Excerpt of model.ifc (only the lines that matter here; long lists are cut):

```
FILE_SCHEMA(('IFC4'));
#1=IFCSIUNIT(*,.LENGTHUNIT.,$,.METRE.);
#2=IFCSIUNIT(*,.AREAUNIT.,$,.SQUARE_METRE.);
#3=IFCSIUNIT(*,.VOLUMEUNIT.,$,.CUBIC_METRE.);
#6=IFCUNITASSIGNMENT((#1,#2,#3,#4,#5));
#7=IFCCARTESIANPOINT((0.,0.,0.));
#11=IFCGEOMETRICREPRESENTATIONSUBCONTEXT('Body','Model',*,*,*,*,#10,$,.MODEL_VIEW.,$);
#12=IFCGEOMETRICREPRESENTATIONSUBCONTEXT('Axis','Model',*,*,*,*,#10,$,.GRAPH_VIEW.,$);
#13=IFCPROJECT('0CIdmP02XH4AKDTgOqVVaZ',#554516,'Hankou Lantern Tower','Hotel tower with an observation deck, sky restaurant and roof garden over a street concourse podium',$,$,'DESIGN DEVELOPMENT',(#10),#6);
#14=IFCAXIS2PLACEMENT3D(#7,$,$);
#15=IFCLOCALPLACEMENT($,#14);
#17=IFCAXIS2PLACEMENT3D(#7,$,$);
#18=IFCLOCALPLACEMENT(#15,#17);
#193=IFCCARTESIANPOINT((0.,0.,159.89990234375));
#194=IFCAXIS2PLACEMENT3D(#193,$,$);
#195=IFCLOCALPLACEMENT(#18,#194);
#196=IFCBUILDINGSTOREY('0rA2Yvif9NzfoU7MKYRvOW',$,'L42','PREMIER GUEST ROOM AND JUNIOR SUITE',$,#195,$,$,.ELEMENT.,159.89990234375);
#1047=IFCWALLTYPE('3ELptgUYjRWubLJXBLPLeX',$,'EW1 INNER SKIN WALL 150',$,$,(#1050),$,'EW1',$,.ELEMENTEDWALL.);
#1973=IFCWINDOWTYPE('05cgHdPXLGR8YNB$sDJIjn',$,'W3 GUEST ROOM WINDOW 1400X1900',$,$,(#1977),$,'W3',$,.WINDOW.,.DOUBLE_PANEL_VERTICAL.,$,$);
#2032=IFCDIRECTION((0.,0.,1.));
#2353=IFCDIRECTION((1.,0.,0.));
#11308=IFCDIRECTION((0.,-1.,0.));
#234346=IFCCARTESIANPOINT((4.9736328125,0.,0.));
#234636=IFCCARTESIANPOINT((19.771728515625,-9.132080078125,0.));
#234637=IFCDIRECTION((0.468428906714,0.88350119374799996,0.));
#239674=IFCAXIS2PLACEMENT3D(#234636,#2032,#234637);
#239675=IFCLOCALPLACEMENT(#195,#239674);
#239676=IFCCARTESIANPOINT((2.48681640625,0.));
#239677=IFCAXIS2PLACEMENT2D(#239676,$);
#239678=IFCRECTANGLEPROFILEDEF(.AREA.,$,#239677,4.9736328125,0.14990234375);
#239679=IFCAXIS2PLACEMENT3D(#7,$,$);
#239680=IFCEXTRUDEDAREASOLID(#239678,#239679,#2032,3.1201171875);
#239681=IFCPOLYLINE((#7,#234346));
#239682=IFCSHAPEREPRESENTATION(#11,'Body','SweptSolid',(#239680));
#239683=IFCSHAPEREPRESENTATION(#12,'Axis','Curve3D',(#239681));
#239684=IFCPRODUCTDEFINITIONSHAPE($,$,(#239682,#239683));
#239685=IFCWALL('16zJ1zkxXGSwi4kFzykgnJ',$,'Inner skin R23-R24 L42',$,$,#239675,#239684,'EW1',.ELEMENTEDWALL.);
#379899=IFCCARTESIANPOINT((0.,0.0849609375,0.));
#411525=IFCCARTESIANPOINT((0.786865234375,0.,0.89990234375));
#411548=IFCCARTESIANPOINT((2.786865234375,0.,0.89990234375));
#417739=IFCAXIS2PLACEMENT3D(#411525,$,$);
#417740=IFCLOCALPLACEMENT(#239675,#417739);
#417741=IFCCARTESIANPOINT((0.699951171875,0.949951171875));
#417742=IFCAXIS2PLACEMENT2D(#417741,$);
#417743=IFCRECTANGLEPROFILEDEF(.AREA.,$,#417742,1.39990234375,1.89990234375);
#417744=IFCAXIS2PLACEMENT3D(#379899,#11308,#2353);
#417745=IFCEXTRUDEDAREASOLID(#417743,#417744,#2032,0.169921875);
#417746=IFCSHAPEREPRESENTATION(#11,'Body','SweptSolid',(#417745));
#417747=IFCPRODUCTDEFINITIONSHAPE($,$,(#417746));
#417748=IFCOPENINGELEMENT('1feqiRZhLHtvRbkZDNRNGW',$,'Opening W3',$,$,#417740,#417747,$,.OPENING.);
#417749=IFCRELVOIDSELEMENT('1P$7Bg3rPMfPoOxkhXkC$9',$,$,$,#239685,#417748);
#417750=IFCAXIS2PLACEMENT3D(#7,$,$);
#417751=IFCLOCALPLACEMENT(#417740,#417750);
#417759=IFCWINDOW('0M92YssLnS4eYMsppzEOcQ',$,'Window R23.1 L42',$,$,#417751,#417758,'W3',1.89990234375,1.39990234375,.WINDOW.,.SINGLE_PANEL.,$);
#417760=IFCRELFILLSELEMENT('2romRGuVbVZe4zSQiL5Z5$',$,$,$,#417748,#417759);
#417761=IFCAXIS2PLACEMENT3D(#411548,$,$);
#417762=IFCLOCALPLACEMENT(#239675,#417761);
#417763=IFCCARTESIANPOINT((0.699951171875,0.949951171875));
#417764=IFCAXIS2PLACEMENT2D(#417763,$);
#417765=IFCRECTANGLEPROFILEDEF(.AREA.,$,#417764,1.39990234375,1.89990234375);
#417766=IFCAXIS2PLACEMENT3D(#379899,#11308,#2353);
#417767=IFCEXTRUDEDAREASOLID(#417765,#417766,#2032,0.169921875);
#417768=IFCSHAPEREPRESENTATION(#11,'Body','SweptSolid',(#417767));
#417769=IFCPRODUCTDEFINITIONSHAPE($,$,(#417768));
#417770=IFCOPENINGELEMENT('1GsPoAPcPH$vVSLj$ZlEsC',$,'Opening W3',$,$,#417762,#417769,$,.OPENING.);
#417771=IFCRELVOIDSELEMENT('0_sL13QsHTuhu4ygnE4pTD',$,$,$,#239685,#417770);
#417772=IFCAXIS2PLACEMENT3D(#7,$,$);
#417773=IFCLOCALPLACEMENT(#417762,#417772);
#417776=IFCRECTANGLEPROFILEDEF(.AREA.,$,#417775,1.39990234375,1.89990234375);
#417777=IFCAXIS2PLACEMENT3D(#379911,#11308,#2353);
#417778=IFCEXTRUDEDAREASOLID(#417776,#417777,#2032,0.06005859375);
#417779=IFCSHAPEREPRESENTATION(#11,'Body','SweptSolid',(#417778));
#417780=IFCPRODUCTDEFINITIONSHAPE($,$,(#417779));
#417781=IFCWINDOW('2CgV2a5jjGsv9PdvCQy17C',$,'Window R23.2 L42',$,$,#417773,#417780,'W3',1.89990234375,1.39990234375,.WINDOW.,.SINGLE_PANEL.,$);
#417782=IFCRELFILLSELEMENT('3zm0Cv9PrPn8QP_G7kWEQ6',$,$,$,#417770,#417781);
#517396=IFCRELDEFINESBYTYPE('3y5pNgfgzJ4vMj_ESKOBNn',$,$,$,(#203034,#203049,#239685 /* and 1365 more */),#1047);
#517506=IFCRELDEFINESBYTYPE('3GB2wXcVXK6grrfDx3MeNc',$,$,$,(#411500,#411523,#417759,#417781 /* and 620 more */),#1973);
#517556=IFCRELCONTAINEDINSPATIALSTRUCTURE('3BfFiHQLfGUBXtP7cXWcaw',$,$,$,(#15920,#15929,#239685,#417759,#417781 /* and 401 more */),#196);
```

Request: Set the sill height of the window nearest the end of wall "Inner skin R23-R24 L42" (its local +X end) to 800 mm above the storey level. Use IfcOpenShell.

```python
import numpy as np
import ifcopenshell
import ifcopenshell.api.geometry
import ifcopenshell.geom
import ifcopenshell.util.element
import ifcopenshell.util.placement
import ifcopenshell.util.shape
import ifcopenshell.util.unit

model = ifcopenshell.open("model.ifc")
unit_scale = ifcopenshell.util.unit.calculate_unit_scale(model)

window = model.by_guid("2CgV2a5jjGsv9PdvCQy17C")
opening = window.FillsVoids[0].RelatingOpeningElement
storey = ifcopenshell.util.element.get_container(window, ifc_class="IfcBuildingStorey")
level = ifcopenshell.util.placement.get_local_placement(storey.ObjectPlacement)[2, 3]

# The opening's origin need not be at the sill, so measure its lowest point.
shape = ifcopenshell.geom.create_shape(ifcopenshell.geom.settings(), opening)
bottom = ifcopenshell.util.shape.get_shape_bottom_elevation(shape, shape.geometry) / unit_scale
dz = level + 0.8 - bottom

shift = np.array([0.0, 0.0, dz])
# The window is placed relative to its opening, so it follows when the opening moves.
matrix = ifcopenshell.util.placement.get_local_placement(opening.ObjectPlacement)
matrix[:3, 3] += shift
ifcopenshell.api.geometry.edit_object_placement(
    model, product=opening, matrix=matrix, is_si=False, should_transform_children=True
)

print(f"moved by {dz * unit_scale:+.3f} m")

model.write("model_v2.ifc")
```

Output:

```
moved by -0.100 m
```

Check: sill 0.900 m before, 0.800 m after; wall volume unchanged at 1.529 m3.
